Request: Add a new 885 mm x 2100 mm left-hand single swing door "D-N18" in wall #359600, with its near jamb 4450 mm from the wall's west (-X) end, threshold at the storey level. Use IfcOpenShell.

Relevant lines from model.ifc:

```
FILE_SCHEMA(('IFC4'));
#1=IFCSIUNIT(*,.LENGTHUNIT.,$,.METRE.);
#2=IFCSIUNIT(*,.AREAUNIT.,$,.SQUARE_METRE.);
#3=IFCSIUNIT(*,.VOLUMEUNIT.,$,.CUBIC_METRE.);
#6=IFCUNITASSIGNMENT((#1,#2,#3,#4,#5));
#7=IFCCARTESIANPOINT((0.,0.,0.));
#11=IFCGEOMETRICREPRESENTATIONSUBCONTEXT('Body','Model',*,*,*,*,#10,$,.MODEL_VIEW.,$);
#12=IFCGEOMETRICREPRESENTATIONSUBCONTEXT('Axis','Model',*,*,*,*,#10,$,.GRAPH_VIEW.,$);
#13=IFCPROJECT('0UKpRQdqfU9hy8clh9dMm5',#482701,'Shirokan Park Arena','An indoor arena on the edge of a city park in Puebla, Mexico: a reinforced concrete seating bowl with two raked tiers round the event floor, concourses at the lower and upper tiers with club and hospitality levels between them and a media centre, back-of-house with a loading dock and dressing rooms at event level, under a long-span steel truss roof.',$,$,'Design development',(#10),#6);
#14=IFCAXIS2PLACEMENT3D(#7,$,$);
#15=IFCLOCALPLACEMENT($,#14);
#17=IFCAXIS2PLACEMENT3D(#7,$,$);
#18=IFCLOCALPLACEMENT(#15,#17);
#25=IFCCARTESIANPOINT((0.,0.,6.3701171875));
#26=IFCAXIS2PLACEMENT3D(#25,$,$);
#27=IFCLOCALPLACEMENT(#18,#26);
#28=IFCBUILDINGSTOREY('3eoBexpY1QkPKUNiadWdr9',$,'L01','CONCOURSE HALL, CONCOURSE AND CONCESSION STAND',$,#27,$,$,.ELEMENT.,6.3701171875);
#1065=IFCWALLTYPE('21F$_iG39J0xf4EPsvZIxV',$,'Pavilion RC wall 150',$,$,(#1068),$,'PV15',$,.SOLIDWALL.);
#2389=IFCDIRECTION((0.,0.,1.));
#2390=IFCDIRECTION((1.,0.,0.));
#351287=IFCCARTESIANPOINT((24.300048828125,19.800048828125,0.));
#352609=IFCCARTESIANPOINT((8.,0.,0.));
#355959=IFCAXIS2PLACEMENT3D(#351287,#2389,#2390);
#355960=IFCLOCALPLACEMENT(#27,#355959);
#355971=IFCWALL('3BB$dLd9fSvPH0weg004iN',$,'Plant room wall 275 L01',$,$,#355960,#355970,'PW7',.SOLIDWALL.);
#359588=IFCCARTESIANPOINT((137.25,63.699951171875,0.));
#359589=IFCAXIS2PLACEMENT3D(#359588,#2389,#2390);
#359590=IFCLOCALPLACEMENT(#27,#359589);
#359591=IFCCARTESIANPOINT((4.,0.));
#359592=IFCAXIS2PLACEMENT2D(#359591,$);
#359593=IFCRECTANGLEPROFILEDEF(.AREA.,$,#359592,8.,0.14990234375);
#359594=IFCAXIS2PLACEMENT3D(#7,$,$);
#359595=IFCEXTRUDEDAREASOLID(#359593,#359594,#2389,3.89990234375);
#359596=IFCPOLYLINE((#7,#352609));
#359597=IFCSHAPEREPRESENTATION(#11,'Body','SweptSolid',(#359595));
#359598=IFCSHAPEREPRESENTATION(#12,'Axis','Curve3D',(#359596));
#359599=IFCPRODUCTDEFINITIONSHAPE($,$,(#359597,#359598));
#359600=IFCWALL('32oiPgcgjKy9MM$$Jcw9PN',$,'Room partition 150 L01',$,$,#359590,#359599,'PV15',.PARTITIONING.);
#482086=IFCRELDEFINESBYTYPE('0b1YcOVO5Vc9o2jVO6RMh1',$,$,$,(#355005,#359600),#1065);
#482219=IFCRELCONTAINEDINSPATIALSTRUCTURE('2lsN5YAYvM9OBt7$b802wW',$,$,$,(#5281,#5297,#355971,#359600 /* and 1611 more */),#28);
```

```python
import numpy as np
import ifcopenshell
import ifcopenshell.api.feature
import ifcopenshell.api.geometry
import ifcopenshell.api.root
import ifcopenshell.api.spatial
import ifcopenshell.geom
import ifcopenshell.util.element
import ifcopenshell.util.placement
import ifcopenshell.util.representation
import ifcopenshell.util.shape
import ifcopenshell.util.unit

model = ifcopenshell.open("model.ifc")
unit_scale = ifcopenshell.util.unit.calculate_unit_scale(model)
settings = ifcopenshell.geom.settings()


def volume(element):
    """Net volume in cubic metres, openings subtracted."""
    shape = ifcopenshell.geom.create_shape(settings, element)
    return ifcopenshell.util.shape.get_volume(shape.geometry)


wall = model.by_guid("32oiPgcgjKy9MM$$Jcw9PN")
storey = ifcopenshell.util.element.get_container(wall, ifc_class="IfcBuildingStorey")
context = ifcopenshell.util.representation.get_context(model, "Model", "Body", "MODEL_VIEW")
before = volume(wall)

width, height, from_end, sill = 0.885, 2.1, 4.45, 0.0  # metres

# The wall runs along its own X axis, and the end named is its -X end.
wall_shape = ifcopenshell.geom.create_shape(settings, wall)
x, y, z = ifcopenshell.util.shape.get_vertices(wall_shape.geometry).T
start = x.min() + from_end
face, thickness = float(y.min()), float(y.max() - y.min())
wall_matrix = ifcopenshell.util.placement.get_local_placement(wall.ObjectPlacement)
level = ifcopenshell.util.placement.get_local_placement(storey.ObjectPlacement)[2, 3]


def in_wall(x, y):
    """Placement at x, y metres in the wall's axes, at sill height."""
    matrix = wall_matrix.copy()
    matrix[:, 3] = wall_matrix @ np.array([x / unit_scale, y / unit_scale, 0.0, 1.0])
    matrix[2, 3] = level + sill / unit_scale
    return matrix


# Opening: a box that overshoots both wall faces by 50 mm.
opening = ifcopenshell.api.root.create_entity(model, ifc_class="IfcOpeningElement", predefined_type="OPENING")
box = ifcopenshell.api.geometry.add_wall_representation(
    model, context=context, length=width, height=height, thickness=thickness + 0.1
)
ifcopenshell.api.geometry.assign_representation(model, product=opening, representation=box)
ifcopenshell.api.geometry.edit_object_placement(model, product=opening, matrix=in_wall(start, face - 0.05), is_si=False)
ifcopenshell.api.feature.add_feature(model, feature=opening, element=wall)

door = ifcopenshell.api.root.create_entity(model, ifc_class="IfcDoor", name="D-N18", predefined_type="DOOR")
door.OverallWidth, door.OverallHeight = width / unit_scale, height / unit_scale
door.OperationType = "SINGLE_SWING_LEFT"
body = ifcopenshell.api.geometry.add_door_representation(
    model,
    context=context,
    overall_width=door.OverallWidth,
    overall_height=door.OverallHeight,
    operation_type="SINGLE_SWING_LEFT",
    lining_properties={"LiningDepth": thickness / unit_scale, "ThresholdDepth": thickness / unit_scale},
)
ifcopenshell.api.geometry.assign_representation(model, product=door, representation=body)
ifcopenshell.api.spatial.assign_container(model, products=[door], relating_structure=storey)
ifcopenshell.api.feature.add_filling(model, opening=opening, element=door)

# The lining spans the wall, so the door starts at the wall face.
ifcopenshell.api.geometry.edit_object_placement(model, product=door, matrix=in_wall(start, face), is_si=False)

after = volume(wall)

print(f"wall volume {before:.3f} -> {after:.3f} m3")

model.write("model_updated.ifc")
```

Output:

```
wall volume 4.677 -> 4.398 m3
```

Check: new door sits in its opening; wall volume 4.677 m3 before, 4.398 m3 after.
